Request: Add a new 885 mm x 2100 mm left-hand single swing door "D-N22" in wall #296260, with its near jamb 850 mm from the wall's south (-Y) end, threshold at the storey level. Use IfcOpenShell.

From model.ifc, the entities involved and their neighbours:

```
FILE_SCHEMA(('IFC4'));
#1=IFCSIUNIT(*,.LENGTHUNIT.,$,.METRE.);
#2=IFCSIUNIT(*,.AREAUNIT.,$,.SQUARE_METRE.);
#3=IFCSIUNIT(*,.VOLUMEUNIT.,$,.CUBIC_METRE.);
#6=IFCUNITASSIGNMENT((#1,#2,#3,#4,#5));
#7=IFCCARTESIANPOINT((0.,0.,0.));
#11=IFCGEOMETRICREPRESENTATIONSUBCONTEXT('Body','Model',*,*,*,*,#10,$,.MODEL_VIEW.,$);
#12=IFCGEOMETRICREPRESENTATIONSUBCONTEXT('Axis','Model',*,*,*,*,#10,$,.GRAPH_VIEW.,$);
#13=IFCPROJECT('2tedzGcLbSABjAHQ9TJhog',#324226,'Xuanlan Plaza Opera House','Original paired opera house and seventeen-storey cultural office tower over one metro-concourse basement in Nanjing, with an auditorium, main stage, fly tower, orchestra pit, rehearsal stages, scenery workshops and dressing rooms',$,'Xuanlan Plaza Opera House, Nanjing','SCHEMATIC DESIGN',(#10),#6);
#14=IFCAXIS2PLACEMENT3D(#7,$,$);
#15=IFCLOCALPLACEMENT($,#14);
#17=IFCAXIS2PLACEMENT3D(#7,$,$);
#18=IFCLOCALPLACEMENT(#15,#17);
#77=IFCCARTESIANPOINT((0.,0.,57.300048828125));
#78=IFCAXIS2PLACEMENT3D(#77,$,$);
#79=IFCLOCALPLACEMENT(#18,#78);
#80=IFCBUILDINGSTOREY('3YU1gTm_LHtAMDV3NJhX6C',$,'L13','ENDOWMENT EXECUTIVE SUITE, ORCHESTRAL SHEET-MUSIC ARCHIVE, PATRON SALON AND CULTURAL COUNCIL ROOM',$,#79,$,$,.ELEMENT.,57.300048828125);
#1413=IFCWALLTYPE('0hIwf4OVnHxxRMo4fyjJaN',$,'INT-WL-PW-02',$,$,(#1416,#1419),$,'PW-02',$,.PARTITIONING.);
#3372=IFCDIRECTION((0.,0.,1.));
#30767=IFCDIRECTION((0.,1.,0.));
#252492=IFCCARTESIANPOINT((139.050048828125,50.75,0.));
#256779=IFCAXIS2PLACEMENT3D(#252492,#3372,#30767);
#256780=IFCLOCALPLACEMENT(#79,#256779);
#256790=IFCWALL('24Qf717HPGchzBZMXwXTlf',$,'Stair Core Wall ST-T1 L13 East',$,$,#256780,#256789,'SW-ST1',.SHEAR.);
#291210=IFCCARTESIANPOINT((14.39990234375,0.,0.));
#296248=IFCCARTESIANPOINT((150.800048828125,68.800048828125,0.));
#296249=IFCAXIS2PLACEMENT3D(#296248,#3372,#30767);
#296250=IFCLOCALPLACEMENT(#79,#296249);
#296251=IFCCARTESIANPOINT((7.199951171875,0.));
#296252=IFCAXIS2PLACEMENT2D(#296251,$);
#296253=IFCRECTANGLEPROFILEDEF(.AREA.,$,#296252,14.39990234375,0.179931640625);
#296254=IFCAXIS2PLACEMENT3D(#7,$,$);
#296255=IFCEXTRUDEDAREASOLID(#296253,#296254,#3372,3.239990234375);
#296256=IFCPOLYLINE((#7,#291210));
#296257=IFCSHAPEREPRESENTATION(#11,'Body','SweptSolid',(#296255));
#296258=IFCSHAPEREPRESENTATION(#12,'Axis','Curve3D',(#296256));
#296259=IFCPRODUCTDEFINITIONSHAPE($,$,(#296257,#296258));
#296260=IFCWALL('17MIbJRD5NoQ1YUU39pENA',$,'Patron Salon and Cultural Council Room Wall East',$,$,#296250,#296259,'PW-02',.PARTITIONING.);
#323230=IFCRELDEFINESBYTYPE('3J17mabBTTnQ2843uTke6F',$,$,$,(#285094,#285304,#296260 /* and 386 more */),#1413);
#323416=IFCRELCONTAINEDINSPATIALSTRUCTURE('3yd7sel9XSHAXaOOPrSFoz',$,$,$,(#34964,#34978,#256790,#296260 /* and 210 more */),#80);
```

```python
import numpy as np
import ifcopenshell
import ifcopenshell.api.feature
import ifcopenshell.api.geometry
import ifcopenshell.api.root
import ifcopenshell.api.spatial
import ifcopenshell.geom
import ifcopenshell.util.element
import ifcopenshell.util.placement
import ifcopenshell.util.representation
import ifcopenshell.util.shape
import ifcopenshell.util.unit

model = ifcopenshell.open("model.ifc")
unit_scale = ifcopenshell.util.unit.calculate_unit_scale(model)
settings = ifcopenshell.geom.settings()


def volume(element):
    """Net volume in cubic metres, openings subtracted."""
    shape = ifcopenshell.geom.create_shape(settings, element)
    return ifcopenshell.util.shape.get_volume(shape.geometry)


wall = model.by_id(296260)
storey = ifcopenshell.util.element.get_container(wall, ifc_class="IfcBuildingStorey")
context = ifcopenshell.util.representation.get_context(model, "Model", "Body", "MODEL_VIEW")
before = volume(wall)

width, height, from_end, sill = 0.885, 2.1, 0.85, 0.0  # metres

# The wall runs along its own X axis, and the end named is its -X end.
wall_shape = ifcopenshell.geom.create_shape(settings, wall)
x, y, z = ifcopenshell.util.shape.get_vertices(wall_shape.geometry).T
start = x.min() + from_end
face, thickness = float(y.min()), float(y.max() - y.min())
wall_matrix = ifcopenshell.util.placement.get_local_placement(wall.ObjectPlacement)
level = ifcopenshell.util.placement.get_local_placement(storey.ObjectPlacement)[2, 3]


def in_wall(x, y):
    """Placement at x, y metres in the wall's axes, at sill height."""
    matrix = wall_matrix.copy()
    matrix[:, 3] = wall_matrix @ np.array([x / unit_scale, y / unit_scale, 0.0, 1.0])
    matrix[2, 3] = level + sill / unit_scale
    return matrix


# Opening: a box that overshoots both wall faces by 50 mm.
opening = ifcopenshell.api.root.create_entity(model, ifc_class="IfcOpeningElement", predefined_type="OPENING")
box = ifcopenshell.api.geometry.add_wall_representation(
    model, context=context, length=width, height=height, thickness=thickness + 0.1
)
ifcopenshell.api.geometry.assign_representation(model, product=opening, representation=box)
ifcopenshell.api.geometry.edit_object_placement(model, product=opening, matrix=in_wall(start, face - 0.05), is_si=False)
ifcopenshell.api.feature.add_feature(model, feature=opening, element=wall)

door = ifcopenshell.api.root.create_entity(model, ifc_class="IfcDoor", name="D-N22", predefined_type="DOOR")
door.OverallWidth, door.OverallHeight = width / unit_scale, height / unit_scale
door.OperationType = "SINGLE_SWING_LEFT"
body = ifcopenshell.api.geometry.add_door_representation(
    model,
    context=context,
    overall_width=door.OverallWidth,
    overall_height=door.OverallHeight,
    operation_type="SINGLE_SWING_LEFT",
    lining_properties={"LiningDepth": thickness / unit_scale, "ThresholdDepth": thickness / unit_scale},
)
ifcopenshell.api.geometry.assign_representation(model, product=door, representation=body)
ifcopenshell.api.spatial.assign_container(model, products=[door], relating_structure=storey)
ifcopenshell.api.feature.add_filling(model, opening=opening, element=door)

# The lining spans the wall, so the door starts at the wall face.
ifcopenshell.api.geometry.edit_object_placement(model, product=door, matrix=in_wall(start, face), is_si=False)

after = volume(wall)

print(f"wall volume {before:.3f} -> {after:.3f} m3")

model.write("model-out.ifc")
```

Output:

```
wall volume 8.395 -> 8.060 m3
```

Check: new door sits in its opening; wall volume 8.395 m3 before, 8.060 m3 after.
